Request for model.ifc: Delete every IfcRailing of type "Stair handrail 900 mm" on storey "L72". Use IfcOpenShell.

First a look at what the model holds.

```python
import ifcopenshell
import ifcopenshell.util.element

model = ifcopenshell.open("model.ifc")
print(model.schema)
storey = next(s for s in model.by_type("IfcBuildingStorey") if s.Name == "L72")
railings = [e for e in ifcopenshell.util.element.get_decomposition(storey) if e.is_a("IfcRailing")]
seen = {}
for e in railings:
    element_type = ifcopenshell.util.element.get_type(e)
    name = element_type.Name if element_type not in (None, e) else None
    seen[name] = seen.get(name, 0) + 1
for name, count in sorted(seen.items(), key=str):
    print(count, "x", name)
```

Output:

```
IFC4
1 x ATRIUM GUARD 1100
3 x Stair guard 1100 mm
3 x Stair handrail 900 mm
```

```python
import ifcopenshell
import ifcopenshell.api.root
import ifcopenshell.util.element

model = ifcopenshell.open("model.ifc")

storey = next(s for s in model.by_type("IfcBuildingStorey") if s.Name == "L72")
railings = [e for e in ifcopenshell.util.element.get_decomposition(storey) if e.is_a("IfcRailing")]
targets = [e for e in railings if (t := ifcopenshell.util.element.get_type(e)) not in (None, e) and t.Name == "Stair handrail 900 mm"]

for e in targets:
    ifcopenshell.api.root.remove_product(model, product=e)
print(len(targets), "removed")

model.write("model_updated.ifc")
```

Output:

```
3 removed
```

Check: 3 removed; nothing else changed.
